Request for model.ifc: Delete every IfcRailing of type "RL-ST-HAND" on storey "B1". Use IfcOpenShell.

First a look at what the model holds.

```python
import ifcopenshell
import ifcopenshell.util.element

model = ifcopenshell.open("model.ifc")
print(model.schema)
storey = next(s for s in model.by_type("IfcBuildingStorey") if s.Name == "B1")
railings = [e for e in ifcopenshell.util.element.get_decomposition(storey) if e.is_a("IfcRailing")]
seen = {}
for e in railings:
    element_type = ifcopenshell.util.element.get_type(e)
    name = element_type.Name if element_type not in (None, e) else None
    seen[name] = seen.get(name, 0) + 1
for name, count in sorted(seen.items(), key=str):
    print(count, "x", name)
```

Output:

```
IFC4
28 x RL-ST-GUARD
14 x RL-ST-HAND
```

```python
import ifcopenshell
import ifcopenshell.api.root
import ifcopenshell.util.element

model = ifcopenshell.open("model.ifc")

storey = next(s for s in model.by_type("IfcBuildingStorey") if s.Name == "B1")
railings = [e for e in ifcopenshell.util.element.get_decomposition(storey) if e.is_a("IfcRailing")]
targets = [e for e in railings if (t := ifcopenshell.util.element.get_type(e)) not in (None, e) and t.Name == "RL-ST-HAND"]

for e in targets:
    ifcopenshell.api.root.remove_product(model, product=e)
print(len(targets), "removed")

model.write("model_v2.ifc")
```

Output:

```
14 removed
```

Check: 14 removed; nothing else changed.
